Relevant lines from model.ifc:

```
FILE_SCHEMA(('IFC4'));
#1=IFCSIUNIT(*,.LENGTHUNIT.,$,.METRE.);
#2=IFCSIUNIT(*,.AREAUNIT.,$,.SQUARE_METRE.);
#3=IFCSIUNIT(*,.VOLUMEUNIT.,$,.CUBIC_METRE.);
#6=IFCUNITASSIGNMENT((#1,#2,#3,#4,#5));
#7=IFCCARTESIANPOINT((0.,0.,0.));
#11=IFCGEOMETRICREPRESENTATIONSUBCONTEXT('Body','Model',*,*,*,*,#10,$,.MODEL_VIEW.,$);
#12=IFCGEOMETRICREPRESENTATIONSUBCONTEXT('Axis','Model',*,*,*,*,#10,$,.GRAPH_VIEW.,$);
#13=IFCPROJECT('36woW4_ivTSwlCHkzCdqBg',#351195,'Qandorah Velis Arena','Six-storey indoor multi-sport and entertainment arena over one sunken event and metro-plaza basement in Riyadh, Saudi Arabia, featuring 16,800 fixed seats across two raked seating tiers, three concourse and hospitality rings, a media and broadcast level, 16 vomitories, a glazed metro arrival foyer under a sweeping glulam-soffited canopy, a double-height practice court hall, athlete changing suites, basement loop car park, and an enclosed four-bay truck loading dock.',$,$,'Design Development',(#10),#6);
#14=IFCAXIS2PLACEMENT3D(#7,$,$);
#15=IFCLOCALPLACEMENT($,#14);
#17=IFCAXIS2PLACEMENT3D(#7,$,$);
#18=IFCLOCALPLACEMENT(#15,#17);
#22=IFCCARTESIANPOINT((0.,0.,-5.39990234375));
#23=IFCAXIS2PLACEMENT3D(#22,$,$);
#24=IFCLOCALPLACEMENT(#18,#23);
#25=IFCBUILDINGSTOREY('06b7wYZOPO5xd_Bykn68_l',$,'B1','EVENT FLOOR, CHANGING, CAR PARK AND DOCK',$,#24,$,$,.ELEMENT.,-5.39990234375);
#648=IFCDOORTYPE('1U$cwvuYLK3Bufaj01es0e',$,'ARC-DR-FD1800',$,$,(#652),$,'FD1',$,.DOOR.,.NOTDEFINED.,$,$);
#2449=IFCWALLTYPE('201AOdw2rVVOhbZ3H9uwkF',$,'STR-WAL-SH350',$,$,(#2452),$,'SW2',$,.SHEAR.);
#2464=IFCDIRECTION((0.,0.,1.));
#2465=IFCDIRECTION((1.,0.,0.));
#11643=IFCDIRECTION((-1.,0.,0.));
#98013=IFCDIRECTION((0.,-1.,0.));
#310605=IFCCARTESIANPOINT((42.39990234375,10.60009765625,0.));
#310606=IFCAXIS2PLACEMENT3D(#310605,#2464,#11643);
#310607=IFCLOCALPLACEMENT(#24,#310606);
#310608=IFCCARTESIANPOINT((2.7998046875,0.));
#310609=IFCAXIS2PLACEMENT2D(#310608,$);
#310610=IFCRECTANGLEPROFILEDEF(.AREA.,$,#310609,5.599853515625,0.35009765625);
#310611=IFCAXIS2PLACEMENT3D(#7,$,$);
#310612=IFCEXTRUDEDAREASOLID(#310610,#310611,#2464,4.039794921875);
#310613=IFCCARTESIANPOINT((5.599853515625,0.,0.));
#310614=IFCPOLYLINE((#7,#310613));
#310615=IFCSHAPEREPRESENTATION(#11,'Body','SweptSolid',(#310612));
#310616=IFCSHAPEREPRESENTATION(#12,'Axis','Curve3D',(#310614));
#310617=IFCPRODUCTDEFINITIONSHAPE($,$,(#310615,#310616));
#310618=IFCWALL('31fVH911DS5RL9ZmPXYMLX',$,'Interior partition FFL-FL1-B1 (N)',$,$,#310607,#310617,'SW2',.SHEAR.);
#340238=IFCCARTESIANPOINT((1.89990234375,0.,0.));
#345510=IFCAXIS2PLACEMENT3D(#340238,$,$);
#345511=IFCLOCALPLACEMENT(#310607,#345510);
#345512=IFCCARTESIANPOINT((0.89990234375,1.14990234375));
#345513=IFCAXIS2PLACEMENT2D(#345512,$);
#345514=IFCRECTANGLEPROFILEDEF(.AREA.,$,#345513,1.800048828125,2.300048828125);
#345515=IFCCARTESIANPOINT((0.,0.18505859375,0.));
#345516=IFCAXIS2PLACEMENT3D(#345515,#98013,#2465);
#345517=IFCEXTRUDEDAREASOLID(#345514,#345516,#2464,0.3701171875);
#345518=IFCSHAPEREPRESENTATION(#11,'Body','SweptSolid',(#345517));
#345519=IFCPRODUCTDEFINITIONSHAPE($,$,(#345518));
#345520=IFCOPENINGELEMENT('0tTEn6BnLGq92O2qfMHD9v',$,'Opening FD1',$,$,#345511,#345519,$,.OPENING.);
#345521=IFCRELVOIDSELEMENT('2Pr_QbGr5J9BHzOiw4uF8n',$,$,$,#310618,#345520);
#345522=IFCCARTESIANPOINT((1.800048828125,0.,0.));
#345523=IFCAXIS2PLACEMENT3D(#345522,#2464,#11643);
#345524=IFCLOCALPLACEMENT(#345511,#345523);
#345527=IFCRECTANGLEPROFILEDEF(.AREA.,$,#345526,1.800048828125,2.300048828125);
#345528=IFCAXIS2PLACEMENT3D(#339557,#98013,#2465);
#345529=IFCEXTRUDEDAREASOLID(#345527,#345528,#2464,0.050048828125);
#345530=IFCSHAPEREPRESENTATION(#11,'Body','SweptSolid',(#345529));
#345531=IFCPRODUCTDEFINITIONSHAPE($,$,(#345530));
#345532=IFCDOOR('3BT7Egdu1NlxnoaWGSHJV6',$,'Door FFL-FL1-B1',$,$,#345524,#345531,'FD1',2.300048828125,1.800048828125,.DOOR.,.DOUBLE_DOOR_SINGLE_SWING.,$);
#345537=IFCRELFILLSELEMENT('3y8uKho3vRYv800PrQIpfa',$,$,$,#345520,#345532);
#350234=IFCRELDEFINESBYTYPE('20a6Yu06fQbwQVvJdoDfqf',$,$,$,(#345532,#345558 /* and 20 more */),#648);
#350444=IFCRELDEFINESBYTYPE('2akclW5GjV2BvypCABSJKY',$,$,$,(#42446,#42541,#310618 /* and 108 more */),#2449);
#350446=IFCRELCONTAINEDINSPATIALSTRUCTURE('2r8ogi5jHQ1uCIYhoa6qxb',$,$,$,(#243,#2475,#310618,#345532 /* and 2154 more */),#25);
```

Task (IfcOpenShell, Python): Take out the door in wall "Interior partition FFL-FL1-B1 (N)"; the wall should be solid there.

```python
import ifcopenshell
import ifcopenshell.api.feature
import ifcopenshell.api.root
import ifcopenshell.geom
import ifcopenshell.util.shape

model = ifcopenshell.open("model.ifc")
settings = ifcopenshell.geom.settings()


def volume(element):
    """Net volume in cubic metres, openings subtracted."""
    shape = ifcopenshell.geom.create_shape(settings, element)
    return ifcopenshell.util.shape.get_volume(shape.geometry)


door = model.by_id(345532)
opening = door.FillsVoids[0].RelatingOpeningElement
wall = opening.VoidsElements[0].RelatingBuildingElement
before = volume(wall)

ifcopenshell.api.root.remove_product(model, product=door)
ifcopenshell.api.feature.remove_feature(model, feature=opening)

after = volume(wall)

print(f"wall volume {before:.3f} -> {after:.3f} m3")

model.write("model_v2.ifc")
```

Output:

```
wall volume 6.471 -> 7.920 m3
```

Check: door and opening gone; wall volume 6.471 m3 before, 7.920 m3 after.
